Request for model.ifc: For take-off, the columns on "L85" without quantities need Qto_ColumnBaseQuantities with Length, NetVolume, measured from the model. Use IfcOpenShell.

First a look at what the model holds.

```python
import ifcopenshell
import ifcopenshell.util.element
import ifcopenshell.util.unit

model = ifcopenshell.open("model.ifc")
print(model.schema)
for unit_type in ("LENGTHUNIT", "AREAUNIT", "VOLUMEUNIT"):
    print(unit_type, ifcopenshell.util.unit.calculate_unit_scale(model, unit_type))
storey = next(s for s in model.by_type("IfcBuildingStorey") if s.Name == "L85")
columns = [e for e in ifcopenshell.util.element.get_decomposition(storey) if e.is_a("IfcColumn")]
for e in sorted(columns, key=lambda e: e.id()):
    print(e.id(), e.is_a(), e.Name, list(ifcopenshell.util.element.get_psets(e, qtos_only=True)), sep=" | ")
```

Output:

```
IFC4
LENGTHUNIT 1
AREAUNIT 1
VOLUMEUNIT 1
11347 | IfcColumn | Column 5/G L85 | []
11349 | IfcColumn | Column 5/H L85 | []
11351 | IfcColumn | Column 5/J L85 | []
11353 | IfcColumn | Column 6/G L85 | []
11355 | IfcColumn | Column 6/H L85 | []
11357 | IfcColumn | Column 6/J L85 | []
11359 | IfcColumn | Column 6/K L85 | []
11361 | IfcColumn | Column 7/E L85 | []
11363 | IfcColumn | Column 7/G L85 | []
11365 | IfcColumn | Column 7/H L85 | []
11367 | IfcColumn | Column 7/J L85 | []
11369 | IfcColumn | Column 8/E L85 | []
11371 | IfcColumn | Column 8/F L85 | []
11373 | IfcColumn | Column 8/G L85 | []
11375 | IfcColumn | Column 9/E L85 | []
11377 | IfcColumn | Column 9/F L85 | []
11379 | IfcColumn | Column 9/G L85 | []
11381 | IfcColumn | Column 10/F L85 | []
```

```python
import ifcopenshell
import ifcopenshell.api.pset
import ifcopenshell.geom
import ifcopenshell.util.element
import ifcopenshell.util.shape
import ifcopenshell.util.unit

model = ifcopenshell.open("model.ifc")
unit_scale = ifcopenshell.util.unit.calculate_unit_scale(model)
volume_scale = ifcopenshell.util.unit.calculate_unit_scale(model, "VOLUMEUNIT")
settings = ifcopenshell.geom.settings()

storey = next(s for s in model.by_type("IfcBuildingStorey") if s.Name == "L85")
columns = [e for e in ifcopenshell.util.element.get_decomposition(storey) if e.is_a("IfcColumn")]

for e in sorted(columns, key=lambda e: e.id()):
    if ifcopenshell.util.element.get_psets(e, qtos_only=True, should_inherit=False):
        continue
    # Geometry comes back in metres, in the element's own axes.
    shape = ifcopenshell.geom.create_shape(settings, e)
    values = {
        "Length": ifcopenshell.util.shape.get_z(shape.geometry) / unit_scale,
        "NetVolume": ifcopenshell.util.shape.get_volume(shape.geometry) / volume_scale,
    }
    qto = ifcopenshell.api.pset.add_qto(model, product=e, name="Qto_ColumnBaseQuantities")
    ifcopenshell.api.pset.edit_qto(model, qto=qto, properties=values)
    print(e.id(), {k: round(v, 3) for k, v in values.items()})

model.write("model_edited.ifc")
```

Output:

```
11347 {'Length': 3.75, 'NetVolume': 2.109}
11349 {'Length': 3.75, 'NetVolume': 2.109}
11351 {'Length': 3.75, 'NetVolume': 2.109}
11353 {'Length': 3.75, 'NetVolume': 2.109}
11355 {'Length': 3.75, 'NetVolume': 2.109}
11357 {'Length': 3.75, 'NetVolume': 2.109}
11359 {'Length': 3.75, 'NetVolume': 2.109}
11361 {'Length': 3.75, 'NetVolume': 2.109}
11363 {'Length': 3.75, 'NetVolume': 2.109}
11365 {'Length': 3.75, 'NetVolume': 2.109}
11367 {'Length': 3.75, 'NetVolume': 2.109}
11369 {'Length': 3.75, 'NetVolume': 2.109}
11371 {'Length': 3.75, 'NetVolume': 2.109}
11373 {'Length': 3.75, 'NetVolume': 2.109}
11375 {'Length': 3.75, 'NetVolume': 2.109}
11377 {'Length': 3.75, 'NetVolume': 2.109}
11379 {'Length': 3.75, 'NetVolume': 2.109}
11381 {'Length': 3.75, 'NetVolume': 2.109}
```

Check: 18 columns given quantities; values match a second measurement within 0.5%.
